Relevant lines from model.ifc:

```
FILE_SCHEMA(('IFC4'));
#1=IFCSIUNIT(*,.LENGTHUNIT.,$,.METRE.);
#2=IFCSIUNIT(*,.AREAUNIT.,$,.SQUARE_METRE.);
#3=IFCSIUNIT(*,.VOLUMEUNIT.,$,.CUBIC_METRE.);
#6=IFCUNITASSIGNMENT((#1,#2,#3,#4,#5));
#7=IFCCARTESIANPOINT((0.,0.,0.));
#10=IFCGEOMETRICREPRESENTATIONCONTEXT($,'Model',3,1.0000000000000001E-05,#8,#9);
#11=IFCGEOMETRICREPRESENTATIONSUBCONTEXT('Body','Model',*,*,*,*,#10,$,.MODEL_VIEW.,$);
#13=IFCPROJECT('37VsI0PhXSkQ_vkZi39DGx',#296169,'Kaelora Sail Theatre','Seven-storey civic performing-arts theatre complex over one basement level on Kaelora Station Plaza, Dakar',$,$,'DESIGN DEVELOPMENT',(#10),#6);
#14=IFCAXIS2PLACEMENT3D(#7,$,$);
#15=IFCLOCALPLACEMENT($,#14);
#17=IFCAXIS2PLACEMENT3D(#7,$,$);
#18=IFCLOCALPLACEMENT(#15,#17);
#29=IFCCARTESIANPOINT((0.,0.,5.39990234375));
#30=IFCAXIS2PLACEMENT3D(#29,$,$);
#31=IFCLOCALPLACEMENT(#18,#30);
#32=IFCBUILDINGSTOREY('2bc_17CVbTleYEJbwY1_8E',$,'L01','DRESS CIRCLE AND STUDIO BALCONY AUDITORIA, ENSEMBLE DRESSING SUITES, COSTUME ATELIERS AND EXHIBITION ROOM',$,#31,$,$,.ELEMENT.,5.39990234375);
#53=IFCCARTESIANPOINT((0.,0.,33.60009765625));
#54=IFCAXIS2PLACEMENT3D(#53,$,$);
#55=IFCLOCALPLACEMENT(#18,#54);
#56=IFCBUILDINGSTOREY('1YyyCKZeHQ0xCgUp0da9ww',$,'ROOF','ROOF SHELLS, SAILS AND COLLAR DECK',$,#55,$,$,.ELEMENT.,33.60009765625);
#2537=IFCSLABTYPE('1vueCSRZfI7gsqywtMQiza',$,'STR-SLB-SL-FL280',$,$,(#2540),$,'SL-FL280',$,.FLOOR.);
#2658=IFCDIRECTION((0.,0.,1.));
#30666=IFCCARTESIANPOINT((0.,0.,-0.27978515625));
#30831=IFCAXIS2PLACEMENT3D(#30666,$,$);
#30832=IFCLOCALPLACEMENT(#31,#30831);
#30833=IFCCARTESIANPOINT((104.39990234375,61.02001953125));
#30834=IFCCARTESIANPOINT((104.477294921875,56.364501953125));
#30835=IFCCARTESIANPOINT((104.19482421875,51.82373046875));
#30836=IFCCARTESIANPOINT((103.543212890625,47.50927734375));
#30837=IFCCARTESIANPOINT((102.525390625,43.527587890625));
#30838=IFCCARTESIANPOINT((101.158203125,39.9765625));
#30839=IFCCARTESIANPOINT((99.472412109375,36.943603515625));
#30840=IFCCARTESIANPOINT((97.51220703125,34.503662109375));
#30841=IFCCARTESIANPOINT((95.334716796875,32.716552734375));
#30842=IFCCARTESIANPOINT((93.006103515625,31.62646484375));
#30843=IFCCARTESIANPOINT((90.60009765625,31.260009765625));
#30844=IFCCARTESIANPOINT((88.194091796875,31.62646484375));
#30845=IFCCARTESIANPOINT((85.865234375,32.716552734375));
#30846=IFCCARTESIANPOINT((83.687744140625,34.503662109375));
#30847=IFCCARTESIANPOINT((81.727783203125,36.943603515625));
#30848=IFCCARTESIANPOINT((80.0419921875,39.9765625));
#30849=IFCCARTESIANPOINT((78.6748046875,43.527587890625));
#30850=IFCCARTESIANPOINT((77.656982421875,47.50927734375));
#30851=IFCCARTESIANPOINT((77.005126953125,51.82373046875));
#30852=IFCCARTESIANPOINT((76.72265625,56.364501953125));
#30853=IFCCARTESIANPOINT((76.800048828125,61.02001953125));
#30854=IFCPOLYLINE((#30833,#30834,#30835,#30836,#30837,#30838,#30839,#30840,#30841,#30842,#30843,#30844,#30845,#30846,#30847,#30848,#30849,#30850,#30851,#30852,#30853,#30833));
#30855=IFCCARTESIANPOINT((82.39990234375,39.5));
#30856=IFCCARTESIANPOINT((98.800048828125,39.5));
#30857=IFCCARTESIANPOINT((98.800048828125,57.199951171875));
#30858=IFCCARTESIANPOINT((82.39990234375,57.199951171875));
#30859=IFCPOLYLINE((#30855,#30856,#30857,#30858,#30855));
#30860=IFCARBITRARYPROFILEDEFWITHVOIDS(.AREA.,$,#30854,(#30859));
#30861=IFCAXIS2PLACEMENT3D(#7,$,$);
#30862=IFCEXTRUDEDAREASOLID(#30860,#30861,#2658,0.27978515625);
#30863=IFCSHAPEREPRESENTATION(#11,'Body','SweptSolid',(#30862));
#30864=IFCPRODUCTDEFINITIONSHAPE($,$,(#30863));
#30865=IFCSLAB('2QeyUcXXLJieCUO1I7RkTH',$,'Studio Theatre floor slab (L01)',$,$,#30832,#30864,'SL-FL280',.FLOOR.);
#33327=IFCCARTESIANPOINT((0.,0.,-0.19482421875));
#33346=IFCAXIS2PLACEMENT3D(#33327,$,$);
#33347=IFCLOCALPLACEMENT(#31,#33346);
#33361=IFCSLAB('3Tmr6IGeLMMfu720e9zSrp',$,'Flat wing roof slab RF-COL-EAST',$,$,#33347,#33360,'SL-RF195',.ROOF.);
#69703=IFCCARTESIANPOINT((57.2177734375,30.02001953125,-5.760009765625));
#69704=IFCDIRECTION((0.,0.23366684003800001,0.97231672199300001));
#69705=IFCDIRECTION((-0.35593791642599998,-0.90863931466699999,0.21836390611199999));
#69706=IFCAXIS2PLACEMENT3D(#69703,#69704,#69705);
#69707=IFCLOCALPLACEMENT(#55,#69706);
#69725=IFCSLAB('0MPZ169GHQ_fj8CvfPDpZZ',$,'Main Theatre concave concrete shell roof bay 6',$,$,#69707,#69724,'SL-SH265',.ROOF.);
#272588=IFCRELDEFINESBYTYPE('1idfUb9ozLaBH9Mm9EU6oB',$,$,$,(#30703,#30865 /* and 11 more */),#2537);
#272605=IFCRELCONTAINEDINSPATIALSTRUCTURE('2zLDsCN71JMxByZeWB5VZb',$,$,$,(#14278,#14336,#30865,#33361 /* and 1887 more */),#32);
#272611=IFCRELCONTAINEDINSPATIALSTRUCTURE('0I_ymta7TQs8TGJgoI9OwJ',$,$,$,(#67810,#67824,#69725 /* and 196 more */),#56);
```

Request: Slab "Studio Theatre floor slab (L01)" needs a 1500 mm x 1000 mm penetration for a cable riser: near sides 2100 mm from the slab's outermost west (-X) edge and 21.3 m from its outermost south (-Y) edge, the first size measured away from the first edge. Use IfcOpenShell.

```python
import numpy as np
import ifcopenshell
import ifcopenshell.api.feature
import ifcopenshell.api.geometry
import ifcopenshell.api.root
import ifcopenshell.geom
import ifcopenshell.util.placement
import ifcopenshell.util.representation
import ifcopenshell.util.shape
import ifcopenshell.util.unit

model = ifcopenshell.open("model.ifc")
unit_scale = ifcopenshell.util.unit.calculate_unit_scale(model)
settings = ifcopenshell.geom.settings()


def volume(element):
    """Net volume in cubic metres, openings subtracted."""
    shape = ifcopenshell.geom.create_shape(settings, element)
    return ifcopenshell.util.shape.get_volume(shape.geometry)


slab = model.by_guid("2QeyUcXXLJieCUO1I7RkTH")
before = volume(slab)

# Extent in the slab's own axes, in metres. The edges named are its -X and -Y sides.
slab_shape = ifcopenshell.geom.create_shape(settings, slab)
vertices = ifcopenshell.util.shape.get_vertices(slab_shape.geometry)
x_min, y_min, bottom = vertices.min(axis=0)
top = vertices[:, 2].max()

opening = ifcopenshell.api.root.create_entity(model, ifc_class="IfcOpeningElement", name="Cable riser opening", predefined_type="OPENING")
context = ifcopenshell.util.representation.get_context(model, "Model", "Body", "MODEL_VIEW")
width, depth = 1.5, 1
outline = [(0.0, 0.0), (width, 0.0), (width, depth), (0.0, depth), (0.0, 0.0)]
# Overshoot both faces by 50 mm so the cut is clean.
shape = ifcopenshell.api.geometry.add_slab_representation(
    model, context=context, depth=top - bottom + 0.1, polyline=outline
)
ifcopenshell.api.geometry.assign_representation(model, product=opening, representation=shape)

matrix = ifcopenshell.util.placement.get_local_placement(slab.ObjectPlacement)
matrix[:, 3] = matrix @ np.append(np.array([x_min + 2.1, y_min + 21.3, bottom - 0.05]) / unit_scale, 1.0)
ifcopenshell.api.geometry.edit_object_placement(model, product=opening, matrix=matrix, is_si=False)
ifcopenshell.api.feature.add_feature(model, feature=opening, element=slab)

after = volume(slab)

print(f"slab volume {before:.3f} -> {after:.3f} m3")

model.write("model-out.ifc")
```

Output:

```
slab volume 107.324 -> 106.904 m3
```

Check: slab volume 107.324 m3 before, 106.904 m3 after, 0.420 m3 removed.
